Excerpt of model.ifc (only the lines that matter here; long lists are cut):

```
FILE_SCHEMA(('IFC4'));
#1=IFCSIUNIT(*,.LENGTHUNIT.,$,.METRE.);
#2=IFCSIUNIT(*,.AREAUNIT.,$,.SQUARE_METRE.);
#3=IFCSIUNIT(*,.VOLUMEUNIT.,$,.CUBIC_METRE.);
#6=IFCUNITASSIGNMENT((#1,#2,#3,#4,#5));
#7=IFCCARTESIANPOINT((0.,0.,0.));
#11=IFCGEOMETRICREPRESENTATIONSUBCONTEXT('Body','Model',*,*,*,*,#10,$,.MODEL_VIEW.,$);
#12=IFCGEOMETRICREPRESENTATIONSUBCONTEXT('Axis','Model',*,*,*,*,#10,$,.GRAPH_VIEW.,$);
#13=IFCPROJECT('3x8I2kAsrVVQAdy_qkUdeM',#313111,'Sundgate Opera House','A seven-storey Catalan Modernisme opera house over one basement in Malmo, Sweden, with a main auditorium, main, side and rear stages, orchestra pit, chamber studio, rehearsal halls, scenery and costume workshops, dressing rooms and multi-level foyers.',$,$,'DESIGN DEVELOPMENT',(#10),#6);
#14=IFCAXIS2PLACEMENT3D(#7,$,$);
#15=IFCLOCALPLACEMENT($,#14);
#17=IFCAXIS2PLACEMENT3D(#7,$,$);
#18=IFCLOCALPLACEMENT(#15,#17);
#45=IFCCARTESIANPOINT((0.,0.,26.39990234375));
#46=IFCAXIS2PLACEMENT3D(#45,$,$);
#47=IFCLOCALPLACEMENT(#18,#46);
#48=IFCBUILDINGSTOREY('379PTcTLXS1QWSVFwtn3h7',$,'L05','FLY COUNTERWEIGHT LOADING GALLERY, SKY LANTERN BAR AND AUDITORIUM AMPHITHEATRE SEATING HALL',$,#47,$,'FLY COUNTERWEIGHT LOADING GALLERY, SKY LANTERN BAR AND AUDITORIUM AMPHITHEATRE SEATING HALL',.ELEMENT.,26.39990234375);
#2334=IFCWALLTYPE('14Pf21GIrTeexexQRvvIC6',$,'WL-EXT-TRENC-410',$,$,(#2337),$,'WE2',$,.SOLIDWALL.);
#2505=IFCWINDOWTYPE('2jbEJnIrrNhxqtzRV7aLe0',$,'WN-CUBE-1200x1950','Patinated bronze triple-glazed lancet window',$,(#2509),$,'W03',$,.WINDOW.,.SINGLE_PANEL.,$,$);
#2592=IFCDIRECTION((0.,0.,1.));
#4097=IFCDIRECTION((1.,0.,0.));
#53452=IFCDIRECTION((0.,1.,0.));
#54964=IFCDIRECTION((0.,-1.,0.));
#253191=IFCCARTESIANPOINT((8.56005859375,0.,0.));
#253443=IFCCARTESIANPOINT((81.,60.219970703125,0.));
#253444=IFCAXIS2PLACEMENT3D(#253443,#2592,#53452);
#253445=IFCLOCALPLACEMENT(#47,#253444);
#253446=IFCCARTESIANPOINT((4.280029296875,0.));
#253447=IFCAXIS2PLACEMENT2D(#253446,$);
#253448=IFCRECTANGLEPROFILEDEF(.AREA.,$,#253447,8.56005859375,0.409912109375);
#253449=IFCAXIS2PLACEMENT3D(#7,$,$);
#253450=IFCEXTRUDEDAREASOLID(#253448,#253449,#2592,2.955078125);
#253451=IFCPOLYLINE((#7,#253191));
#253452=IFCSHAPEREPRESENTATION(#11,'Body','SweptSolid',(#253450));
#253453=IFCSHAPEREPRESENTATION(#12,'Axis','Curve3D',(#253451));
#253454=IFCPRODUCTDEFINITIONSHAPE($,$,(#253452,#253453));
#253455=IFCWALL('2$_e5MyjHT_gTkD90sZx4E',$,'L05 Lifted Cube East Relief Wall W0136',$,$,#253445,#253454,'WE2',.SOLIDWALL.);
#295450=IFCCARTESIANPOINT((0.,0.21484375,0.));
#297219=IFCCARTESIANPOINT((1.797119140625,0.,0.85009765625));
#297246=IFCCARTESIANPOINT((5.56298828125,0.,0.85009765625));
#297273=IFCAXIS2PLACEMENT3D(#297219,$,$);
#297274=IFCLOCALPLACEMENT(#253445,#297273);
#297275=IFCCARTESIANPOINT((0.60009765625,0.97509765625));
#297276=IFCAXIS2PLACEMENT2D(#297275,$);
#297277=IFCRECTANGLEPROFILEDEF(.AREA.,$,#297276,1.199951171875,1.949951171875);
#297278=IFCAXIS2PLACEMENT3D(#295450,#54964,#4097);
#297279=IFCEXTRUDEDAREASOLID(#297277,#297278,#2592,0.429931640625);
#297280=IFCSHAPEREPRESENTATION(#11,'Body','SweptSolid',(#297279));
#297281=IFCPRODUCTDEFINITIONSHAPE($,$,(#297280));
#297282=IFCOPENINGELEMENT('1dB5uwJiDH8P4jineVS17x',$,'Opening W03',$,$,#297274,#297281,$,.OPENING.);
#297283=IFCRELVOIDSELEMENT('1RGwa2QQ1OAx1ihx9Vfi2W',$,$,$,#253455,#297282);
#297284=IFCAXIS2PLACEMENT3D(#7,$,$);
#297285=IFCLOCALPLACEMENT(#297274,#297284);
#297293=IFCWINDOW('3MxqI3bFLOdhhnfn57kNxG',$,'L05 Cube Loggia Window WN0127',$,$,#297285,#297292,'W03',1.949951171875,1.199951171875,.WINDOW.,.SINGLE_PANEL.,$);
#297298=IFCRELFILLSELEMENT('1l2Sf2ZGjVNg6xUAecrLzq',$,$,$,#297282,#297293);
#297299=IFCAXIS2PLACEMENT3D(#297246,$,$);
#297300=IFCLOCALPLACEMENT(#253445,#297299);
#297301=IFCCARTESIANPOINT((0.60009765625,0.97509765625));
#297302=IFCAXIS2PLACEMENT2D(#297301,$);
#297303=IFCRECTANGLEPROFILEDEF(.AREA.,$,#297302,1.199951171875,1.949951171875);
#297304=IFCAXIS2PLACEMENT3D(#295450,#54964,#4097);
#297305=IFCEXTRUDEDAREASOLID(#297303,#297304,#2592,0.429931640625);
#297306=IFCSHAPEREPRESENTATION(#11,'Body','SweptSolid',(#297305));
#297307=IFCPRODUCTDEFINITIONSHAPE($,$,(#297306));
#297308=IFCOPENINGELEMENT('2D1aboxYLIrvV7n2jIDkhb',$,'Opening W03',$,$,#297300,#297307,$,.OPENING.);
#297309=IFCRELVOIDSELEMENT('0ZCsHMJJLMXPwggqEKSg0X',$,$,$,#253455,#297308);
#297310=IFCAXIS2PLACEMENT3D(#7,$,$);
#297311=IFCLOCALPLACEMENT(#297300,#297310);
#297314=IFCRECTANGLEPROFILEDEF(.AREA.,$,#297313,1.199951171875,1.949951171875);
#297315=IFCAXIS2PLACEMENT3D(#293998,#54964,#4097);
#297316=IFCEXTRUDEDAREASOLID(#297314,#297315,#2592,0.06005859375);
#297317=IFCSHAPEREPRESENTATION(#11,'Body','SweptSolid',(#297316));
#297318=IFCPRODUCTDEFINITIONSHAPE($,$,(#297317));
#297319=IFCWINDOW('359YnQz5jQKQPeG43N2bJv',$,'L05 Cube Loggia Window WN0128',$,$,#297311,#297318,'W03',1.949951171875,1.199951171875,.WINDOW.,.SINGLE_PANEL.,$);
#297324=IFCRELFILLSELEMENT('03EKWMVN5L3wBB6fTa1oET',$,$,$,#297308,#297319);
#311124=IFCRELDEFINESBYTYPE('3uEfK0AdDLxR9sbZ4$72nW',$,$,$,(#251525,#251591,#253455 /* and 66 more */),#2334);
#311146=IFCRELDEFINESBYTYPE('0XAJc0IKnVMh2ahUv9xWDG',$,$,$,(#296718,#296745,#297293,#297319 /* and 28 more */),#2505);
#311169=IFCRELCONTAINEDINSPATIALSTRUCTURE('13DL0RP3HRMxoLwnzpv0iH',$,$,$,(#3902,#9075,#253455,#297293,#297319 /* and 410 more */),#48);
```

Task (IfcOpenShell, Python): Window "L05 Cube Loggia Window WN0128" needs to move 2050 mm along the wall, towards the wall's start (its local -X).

```python
import ifcopenshell
import ifcopenshell.api.geometry
import ifcopenshell.util.placement

model = ifcopenshell.open("model.ifc")

window = model.by_guid("359YnQz5jQKQPeG43N2bJv")
opening = window.FillsVoids[0].RelatingOpeningElement
wall = opening.VoidsElements[0].RelatingBuildingElement

wall_matrix = ifcopenshell.util.placement.get_local_placement(wall.ObjectPlacement)
shift = wall_matrix[:3, 0] * -2.05
before = ifcopenshell.util.placement.get_local_placement(window.ObjectPlacement)[:3, 3].copy()

# The window is placed relative to its opening, so it follows when the opening moves.
matrix = ifcopenshell.util.placement.get_local_placement(opening.ObjectPlacement)
matrix[:3, 3] += shift
ifcopenshell.api.geometry.edit_object_placement(
    model, product=opening, matrix=matrix, is_si=False, should_transform_children=True
)

after = ifcopenshell.util.placement.get_local_placement(window.ObjectPlacement)[:3, 3]
print("window moved by", (after - before).round(3) + 0.0)

model.write("model_v2.ifc")
```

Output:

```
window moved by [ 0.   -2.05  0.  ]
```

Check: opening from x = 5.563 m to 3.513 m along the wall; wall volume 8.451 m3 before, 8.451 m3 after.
